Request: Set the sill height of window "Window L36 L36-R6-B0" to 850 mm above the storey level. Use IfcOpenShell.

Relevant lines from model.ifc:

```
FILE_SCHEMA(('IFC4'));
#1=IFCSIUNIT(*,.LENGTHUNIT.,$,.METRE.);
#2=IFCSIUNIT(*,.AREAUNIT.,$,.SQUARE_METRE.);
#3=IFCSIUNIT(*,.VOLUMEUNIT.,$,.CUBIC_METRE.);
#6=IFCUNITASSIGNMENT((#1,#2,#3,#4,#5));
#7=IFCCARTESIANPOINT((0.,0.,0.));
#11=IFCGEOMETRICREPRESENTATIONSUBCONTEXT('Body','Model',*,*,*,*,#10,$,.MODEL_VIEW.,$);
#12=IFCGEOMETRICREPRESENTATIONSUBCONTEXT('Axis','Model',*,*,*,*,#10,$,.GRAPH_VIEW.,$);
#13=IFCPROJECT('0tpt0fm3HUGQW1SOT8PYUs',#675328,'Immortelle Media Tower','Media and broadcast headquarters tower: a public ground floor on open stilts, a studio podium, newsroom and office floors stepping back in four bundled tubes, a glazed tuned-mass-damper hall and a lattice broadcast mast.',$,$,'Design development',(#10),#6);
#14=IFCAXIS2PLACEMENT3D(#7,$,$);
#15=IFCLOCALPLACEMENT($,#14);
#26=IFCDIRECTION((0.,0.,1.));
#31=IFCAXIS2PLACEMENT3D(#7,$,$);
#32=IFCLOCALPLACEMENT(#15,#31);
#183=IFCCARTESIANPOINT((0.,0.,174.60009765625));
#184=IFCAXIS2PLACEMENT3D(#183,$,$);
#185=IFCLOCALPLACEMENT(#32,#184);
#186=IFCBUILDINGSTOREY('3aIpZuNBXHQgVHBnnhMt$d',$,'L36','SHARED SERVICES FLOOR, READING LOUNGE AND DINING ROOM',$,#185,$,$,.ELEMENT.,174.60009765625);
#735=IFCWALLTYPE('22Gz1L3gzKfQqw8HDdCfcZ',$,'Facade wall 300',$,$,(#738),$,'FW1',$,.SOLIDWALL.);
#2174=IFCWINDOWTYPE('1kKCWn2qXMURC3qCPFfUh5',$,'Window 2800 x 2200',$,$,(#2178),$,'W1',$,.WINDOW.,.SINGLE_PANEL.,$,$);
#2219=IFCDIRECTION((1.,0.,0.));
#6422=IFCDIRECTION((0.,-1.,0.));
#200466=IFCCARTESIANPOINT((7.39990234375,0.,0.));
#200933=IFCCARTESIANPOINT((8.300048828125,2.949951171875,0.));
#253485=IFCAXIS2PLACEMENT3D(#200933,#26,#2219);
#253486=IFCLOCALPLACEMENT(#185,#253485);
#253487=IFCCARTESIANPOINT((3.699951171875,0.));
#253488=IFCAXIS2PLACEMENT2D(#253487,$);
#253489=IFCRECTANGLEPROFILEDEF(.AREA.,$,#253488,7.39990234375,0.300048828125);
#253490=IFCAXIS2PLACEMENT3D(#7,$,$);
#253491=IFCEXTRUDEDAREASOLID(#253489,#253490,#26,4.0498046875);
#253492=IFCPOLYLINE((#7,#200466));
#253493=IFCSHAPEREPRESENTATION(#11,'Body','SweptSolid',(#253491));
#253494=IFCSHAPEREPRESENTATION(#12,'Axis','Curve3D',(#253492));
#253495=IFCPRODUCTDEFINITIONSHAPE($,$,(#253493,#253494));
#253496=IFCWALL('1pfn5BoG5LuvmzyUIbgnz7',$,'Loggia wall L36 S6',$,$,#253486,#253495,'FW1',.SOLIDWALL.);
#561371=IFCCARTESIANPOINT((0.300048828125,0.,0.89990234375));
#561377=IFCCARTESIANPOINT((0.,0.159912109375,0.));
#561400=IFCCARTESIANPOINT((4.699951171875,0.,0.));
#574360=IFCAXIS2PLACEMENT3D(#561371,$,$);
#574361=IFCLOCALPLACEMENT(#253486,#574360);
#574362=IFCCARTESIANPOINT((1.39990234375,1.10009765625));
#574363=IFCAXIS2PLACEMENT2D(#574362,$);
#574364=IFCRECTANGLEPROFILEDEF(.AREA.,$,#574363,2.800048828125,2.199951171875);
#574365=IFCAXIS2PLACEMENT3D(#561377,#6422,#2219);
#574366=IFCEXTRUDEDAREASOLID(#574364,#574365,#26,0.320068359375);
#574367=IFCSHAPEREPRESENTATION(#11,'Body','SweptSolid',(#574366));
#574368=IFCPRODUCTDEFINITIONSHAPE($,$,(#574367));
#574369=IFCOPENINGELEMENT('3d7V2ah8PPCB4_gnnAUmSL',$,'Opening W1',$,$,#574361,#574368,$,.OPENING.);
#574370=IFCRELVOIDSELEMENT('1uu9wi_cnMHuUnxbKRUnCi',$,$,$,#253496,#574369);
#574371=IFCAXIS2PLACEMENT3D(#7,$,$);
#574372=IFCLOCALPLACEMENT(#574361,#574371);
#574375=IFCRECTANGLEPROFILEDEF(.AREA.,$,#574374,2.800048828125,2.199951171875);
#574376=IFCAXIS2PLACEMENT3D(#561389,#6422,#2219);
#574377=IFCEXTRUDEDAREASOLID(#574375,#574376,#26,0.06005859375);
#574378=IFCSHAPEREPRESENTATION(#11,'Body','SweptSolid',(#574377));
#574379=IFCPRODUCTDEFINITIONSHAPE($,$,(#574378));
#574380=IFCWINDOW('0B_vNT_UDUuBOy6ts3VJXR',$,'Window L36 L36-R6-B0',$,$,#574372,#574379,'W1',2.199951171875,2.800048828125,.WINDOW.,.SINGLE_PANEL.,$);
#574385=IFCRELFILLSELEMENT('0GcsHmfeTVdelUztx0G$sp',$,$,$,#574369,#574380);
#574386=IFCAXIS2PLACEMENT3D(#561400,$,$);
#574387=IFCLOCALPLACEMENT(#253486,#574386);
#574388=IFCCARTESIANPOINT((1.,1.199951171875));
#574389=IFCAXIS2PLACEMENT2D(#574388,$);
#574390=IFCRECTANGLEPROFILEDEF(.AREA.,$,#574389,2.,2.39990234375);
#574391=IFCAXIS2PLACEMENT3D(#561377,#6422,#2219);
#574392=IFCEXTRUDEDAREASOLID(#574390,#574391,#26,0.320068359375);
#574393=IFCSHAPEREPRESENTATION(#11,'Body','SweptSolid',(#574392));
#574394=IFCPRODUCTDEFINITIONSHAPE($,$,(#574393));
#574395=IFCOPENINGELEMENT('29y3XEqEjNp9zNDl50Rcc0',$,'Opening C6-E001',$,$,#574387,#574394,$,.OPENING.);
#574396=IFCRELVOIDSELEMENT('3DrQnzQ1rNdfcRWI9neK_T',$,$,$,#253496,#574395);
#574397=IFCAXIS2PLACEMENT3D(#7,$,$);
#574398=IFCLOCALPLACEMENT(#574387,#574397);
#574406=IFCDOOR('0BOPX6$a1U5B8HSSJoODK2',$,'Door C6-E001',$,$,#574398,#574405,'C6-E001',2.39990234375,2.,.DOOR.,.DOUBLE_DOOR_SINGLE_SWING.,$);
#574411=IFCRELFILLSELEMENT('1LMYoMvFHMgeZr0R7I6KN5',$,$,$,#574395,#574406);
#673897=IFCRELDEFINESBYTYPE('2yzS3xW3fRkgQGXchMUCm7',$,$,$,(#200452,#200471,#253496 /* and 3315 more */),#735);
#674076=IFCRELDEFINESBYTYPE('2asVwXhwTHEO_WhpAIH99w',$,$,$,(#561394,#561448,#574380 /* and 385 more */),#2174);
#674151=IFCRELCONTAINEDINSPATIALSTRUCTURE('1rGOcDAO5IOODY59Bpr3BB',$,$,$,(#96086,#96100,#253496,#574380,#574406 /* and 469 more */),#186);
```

```python
import numpy as np
import ifcopenshell
import ifcopenshell.api.geometry
import ifcopenshell.geom
import ifcopenshell.util.element
import ifcopenshell.util.placement
import ifcopenshell.util.shape
import ifcopenshell.util.unit

model = ifcopenshell.open("model.ifc")
unit_scale = ifcopenshell.util.unit.calculate_unit_scale(model)

window = model.by_guid("0B_vNT_UDUuBOy6ts3VJXR")
opening = window.FillsVoids[0].RelatingOpeningElement
storey = ifcopenshell.util.element.get_container(window, ifc_class="IfcBuildingStorey")
level = ifcopenshell.util.placement.get_local_placement(storey.ObjectPlacement)[2, 3]

# The opening's origin need not be at the sill, so measure its lowest point.
shape = ifcopenshell.geom.create_shape(ifcopenshell.geom.settings(), opening)
bottom = ifcopenshell.util.shape.get_shape_bottom_elevation(shape, shape.geometry) / unit_scale
dz = level + 0.85 - bottom

shift = np.array([0.0, 0.0, dz])
# The window is placed relative to its opening, so it follows when the opening moves.
matrix = ifcopenshell.util.placement.get_local_placement(opening.ObjectPlacement)
matrix[:3, 3] += shift
ifcopenshell.api.geometry.edit_object_placement(
    model, product=opening, matrix=matrix, is_si=False, should_transform_children=True
)

print(f"moved by {dz * unit_scale:+.3f} m")

model.write("model-out.ifc")
```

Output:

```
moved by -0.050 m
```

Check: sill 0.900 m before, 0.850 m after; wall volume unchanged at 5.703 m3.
